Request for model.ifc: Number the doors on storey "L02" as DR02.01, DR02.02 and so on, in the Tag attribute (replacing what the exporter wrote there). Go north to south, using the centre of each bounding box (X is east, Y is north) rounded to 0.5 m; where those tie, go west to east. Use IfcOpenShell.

First a look at what the model holds.

```python
import ifcopenshell
import ifcopenshell.util.element
import ifcopenshell.util.placement

model = ifcopenshell.open("model.ifc")
print(model.schema)
storey = next(s for s in model.by_type("IfcBuildingStorey") if s.Name == "L02")
doors = [e for e in ifcopenshell.util.element.get_decomposition(storey) if e.is_a("IfcDoor")]
for e in sorted(doors, key=lambda e: e.id()):
    origin = ifcopenshell.util.placement.get_local_placement(e.ObjectPlacement)[:3, 3]
    print(e.id(), e.Tag, e.Name, origin.round(2) + 0.0, sep=" | ")
```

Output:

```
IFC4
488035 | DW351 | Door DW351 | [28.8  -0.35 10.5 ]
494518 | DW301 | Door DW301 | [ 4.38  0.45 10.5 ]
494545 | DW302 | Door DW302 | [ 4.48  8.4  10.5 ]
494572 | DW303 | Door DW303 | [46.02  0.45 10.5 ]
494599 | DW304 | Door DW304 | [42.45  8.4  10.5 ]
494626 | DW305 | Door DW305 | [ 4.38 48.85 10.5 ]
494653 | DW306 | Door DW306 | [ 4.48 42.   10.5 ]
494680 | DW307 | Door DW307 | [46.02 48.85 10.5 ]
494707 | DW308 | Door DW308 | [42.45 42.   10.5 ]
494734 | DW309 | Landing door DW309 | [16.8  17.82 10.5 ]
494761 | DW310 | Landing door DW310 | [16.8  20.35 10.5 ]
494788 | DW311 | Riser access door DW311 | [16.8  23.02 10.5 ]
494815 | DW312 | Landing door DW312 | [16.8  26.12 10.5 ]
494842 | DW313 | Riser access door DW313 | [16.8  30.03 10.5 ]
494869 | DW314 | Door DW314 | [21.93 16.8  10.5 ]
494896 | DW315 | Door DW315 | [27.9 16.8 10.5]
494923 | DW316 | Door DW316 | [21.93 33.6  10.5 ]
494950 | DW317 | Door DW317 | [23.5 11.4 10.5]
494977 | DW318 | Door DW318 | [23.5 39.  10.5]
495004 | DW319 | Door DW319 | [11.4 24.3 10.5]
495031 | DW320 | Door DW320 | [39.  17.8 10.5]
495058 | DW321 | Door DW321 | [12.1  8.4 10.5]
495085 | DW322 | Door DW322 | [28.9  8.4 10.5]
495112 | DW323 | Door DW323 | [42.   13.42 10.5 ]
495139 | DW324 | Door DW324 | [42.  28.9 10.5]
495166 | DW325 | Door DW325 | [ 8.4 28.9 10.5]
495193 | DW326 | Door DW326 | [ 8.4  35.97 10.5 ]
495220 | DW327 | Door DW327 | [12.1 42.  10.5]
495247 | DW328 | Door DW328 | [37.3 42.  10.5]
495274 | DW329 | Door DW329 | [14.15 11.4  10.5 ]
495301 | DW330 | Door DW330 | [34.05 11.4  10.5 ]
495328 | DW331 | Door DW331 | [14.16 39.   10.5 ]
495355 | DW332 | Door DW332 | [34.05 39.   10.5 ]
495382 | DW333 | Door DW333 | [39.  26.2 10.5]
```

```python
import ifcopenshell
import ifcopenshell.geom
import ifcopenshell.util.element
import ifcopenshell.util.shape

model = ifcopenshell.open("model.ifc")
settings = ifcopenshell.geom.settings()
settings.set("use-world-coords", True)


def centre(element):
    shape = ifcopenshell.geom.create_shape(settings, element)
    return ifcopenshell.util.shape.get_bbox_centroid(shape.geometry)


storey = next(s for s in model.by_type("IfcBuildingStorey") if s.Name == "L02")
doors = [e for e in ifcopenshell.util.element.get_decomposition(storey) if e.is_a("IfcDoor")]

# Insertion points can sit at a corner or the storey origin, so sort by the geometry (in metres).
centres = {e: centre(e) for e in doors}
doors.sort(key=lambda e: (-round(centres[e][1] / 0.5), centres[e][0]))

for i, e in enumerate(doors, start=1):
    number = f"DR02.{i:02d}"
    e.Tag = number
    print(e.id(), number)

model.write("model_v2.ifc")
```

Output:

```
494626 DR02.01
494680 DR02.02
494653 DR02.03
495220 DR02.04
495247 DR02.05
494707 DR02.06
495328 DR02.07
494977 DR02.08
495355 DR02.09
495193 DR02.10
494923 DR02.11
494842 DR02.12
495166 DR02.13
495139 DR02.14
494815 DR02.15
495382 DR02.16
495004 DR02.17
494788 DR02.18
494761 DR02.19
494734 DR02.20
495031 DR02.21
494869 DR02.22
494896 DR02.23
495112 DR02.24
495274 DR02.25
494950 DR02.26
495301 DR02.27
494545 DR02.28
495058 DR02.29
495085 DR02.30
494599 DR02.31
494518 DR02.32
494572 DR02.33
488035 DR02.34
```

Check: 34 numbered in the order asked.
